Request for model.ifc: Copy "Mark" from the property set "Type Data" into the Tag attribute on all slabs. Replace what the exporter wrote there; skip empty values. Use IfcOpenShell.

First a look at what the model holds.

```python
import ifcopenshell
import ifcopenshell.util.element

model = ifcopenshell.open("model.ifc")
print(model.schema)
slabs = model.by_type("IfcSlab")
print(len(slabs), "slabs")
for e in slabs[:8]:
    source = ifcopenshell.util.element.get_pset(e, "Type Data", "Mark")
    target = e.Tag
    print(e.id(), repr(source), repr(target), sep=" | ")
```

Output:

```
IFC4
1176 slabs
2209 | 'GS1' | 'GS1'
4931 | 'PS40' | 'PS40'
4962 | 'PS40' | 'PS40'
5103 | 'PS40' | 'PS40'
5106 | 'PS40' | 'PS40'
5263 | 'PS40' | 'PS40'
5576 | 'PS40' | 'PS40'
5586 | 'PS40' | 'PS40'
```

```python
import ifcopenshell
import ifcopenshell.util.element

model = ifcopenshell.open("model.ifc")

count = 0
for e in model.by_type("IfcSlab"):
    value = ifcopenshell.util.element.get_pset(e, "Type Data", "Mark")
    current = e.Tag
    if not value or not value.strip() or current == value:
        continue
    e.Tag = value
    count += 1

print(count, "slabs updated")

model.write("model_v2.ifc")
```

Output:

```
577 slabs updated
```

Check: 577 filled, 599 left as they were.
